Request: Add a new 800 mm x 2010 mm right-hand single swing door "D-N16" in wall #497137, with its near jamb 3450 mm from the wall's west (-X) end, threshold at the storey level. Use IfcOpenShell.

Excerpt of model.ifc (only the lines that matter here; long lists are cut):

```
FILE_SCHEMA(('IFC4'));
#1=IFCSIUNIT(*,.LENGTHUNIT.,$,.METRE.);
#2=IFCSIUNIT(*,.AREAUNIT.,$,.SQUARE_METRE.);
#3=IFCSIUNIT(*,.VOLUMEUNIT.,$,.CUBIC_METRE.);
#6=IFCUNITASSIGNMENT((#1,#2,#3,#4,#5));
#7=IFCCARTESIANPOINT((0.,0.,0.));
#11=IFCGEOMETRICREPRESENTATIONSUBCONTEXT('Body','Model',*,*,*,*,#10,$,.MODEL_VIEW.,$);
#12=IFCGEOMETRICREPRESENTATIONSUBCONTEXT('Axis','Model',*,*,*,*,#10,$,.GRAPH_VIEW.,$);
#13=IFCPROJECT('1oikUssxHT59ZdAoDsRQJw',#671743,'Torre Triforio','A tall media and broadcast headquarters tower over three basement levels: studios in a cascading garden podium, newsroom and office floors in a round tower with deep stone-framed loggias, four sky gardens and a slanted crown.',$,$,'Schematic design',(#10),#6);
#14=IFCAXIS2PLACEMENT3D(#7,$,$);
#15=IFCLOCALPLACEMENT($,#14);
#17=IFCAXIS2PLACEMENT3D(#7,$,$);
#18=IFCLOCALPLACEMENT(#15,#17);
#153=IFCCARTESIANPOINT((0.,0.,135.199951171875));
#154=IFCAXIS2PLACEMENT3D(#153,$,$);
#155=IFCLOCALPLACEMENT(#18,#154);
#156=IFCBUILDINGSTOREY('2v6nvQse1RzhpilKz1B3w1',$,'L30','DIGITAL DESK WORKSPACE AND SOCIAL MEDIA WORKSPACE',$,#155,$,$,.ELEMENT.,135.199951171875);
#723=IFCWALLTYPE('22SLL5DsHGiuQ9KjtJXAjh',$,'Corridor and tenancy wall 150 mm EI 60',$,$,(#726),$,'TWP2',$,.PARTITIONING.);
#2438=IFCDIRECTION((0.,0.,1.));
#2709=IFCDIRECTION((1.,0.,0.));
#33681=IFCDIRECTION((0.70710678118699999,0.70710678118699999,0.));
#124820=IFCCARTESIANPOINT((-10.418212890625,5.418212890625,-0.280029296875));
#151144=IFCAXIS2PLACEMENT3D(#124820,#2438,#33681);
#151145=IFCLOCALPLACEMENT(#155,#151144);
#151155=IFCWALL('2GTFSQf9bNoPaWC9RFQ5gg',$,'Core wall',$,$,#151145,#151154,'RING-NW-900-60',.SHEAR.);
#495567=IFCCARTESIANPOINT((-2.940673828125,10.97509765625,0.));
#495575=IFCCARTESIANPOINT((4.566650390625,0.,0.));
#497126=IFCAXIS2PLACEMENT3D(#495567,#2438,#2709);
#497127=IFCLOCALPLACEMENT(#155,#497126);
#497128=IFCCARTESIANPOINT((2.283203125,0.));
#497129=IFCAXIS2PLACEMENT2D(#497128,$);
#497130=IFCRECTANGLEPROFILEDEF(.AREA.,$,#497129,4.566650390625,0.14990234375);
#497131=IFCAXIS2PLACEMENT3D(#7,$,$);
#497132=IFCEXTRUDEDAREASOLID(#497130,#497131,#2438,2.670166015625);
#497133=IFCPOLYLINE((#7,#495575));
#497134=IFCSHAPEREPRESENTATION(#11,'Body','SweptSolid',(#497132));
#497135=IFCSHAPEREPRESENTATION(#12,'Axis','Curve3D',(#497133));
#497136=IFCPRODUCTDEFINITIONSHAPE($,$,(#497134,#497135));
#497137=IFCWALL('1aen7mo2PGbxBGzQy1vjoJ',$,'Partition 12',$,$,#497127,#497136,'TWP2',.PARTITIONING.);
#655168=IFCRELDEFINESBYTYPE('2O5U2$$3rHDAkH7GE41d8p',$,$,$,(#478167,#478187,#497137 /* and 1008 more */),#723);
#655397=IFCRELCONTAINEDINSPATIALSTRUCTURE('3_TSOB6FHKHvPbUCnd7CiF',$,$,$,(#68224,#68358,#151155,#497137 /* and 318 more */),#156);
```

```python
import numpy as np
import ifcopenshell
import ifcopenshell.api.feature
import ifcopenshell.api.geometry
import ifcopenshell.api.root
import ifcopenshell.api.spatial
import ifcopenshell.geom
import ifcopenshell.util.element
import ifcopenshell.util.placement
import ifcopenshell.util.representation
import ifcopenshell.util.shape
import ifcopenshell.util.unit

model = ifcopenshell.open("model.ifc")
unit_scale = ifcopenshell.util.unit.calculate_unit_scale(model)
settings = ifcopenshell.geom.settings()


def volume(element):
    """Net volume in cubic metres, openings subtracted."""
    shape = ifcopenshell.geom.create_shape(settings, element)
    return ifcopenshell.util.shape.get_volume(shape.geometry)


wall = model.by_guid("1aen7mo2PGbxBGzQy1vjoJ")
storey = ifcopenshell.util.element.get_container(wall, ifc_class="IfcBuildingStorey")
context = ifcopenshell.util.representation.get_context(model, "Model", "Body", "MODEL_VIEW")
before = volume(wall)

width, height, from_end, sill = 0.8, 2.01, 3.45, 0.0  # metres

# The wall runs along its own X axis, and the end named is its -X end.
wall_shape = ifcopenshell.geom.create_shape(settings, wall)
x, y, z = ifcopenshell.util.shape.get_vertices(wall_shape.geometry).T
start = x.min() + from_end
face, thickness = float(y.min()), float(y.max() - y.min())
wall_matrix = ifcopenshell.util.placement.get_local_placement(wall.ObjectPlacement)
level = ifcopenshell.util.placement.get_local_placement(storey.ObjectPlacement)[2, 3]


def in_wall(x, y):
    """Placement at x, y metres in the wall's axes, at sill height."""
    matrix = wall_matrix.copy()
    matrix[:, 3] = wall_matrix @ np.array([x / unit_scale, y / unit_scale, 0.0, 1.0])
    matrix[2, 3] = level + sill / unit_scale
    return matrix


# Opening: a box that overshoots both wall faces by 50 mm.
opening = ifcopenshell.api.root.create_entity(model, ifc_class="IfcOpeningElement", predefined_type="OPENING")
box = ifcopenshell.api.geometry.add_wall_representation(
    model, context=context, length=width, height=height, thickness=thickness + 0.1
)
ifcopenshell.api.geometry.assign_representation(model, product=opening, representation=box)
ifcopenshell.api.geometry.edit_object_placement(model, product=opening, matrix=in_wall(start, face - 0.05), is_si=False)
ifcopenshell.api.feature.add_feature(model, feature=opening, element=wall)

door = ifcopenshell.api.root.create_entity(model, ifc_class="IfcDoor", name="D-N16", predefined_type="DOOR")
door.OverallWidth, door.OverallHeight = width / unit_scale, height / unit_scale
door.OperationType = "SINGLE_SWING_RIGHT"
body = ifcopenshell.api.geometry.add_door_representation(
    model,
    context=context,
    overall_width=door.OverallWidth,
    overall_height=door.OverallHeight,
    operation_type="SINGLE_SWING_RIGHT",
    lining_properties={"LiningDepth": thickness / unit_scale, "ThresholdDepth": thickness / unit_scale},
)
ifcopenshell.api.geometry.assign_representation(model, product=door, representation=body)
ifcopenshell.api.spatial.assign_container(model, products=[door], relating_structure=storey)
ifcopenshell.api.feature.add_filling(model, opening=opening, element=door)

# The lining spans the wall, so the door starts at the wall face.
ifcopenshell.api.geometry.edit_object_placement(model, product=door, matrix=in_wall(start, face), is_si=False)

after = volume(wall)

print(f"wall volume {before:.3f} -> {after:.3f} m3")

model.write("model_v2.ifc")
```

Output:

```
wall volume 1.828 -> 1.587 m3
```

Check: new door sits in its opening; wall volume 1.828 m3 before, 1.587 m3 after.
